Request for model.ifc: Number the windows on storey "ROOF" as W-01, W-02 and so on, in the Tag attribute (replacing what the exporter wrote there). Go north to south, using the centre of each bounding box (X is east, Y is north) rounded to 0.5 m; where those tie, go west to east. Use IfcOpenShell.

First a look at what the model holds.

```python
import ifcopenshell
import ifcopenshell.util.element
import ifcopenshell.util.placement

model = ifcopenshell.open("model.ifc")
print(model.schema)
storey = next(s for s in model.by_type("IfcBuildingStorey") if s.Name == "ROOF")
windows = [e for e in ifcopenshell.util.element.get_decomposition(storey) if e.is_a("IfcWindow")]
for e in sorted(windows, key=lambda e: e.id()):
    origin = ifcopenshell.util.placement.get_local_placement(e.ObjectPlacement)[:3, 3]
    print(e.id(), e.Tag, e.Name, origin.round(2) + 0.0, sep=" | ")
```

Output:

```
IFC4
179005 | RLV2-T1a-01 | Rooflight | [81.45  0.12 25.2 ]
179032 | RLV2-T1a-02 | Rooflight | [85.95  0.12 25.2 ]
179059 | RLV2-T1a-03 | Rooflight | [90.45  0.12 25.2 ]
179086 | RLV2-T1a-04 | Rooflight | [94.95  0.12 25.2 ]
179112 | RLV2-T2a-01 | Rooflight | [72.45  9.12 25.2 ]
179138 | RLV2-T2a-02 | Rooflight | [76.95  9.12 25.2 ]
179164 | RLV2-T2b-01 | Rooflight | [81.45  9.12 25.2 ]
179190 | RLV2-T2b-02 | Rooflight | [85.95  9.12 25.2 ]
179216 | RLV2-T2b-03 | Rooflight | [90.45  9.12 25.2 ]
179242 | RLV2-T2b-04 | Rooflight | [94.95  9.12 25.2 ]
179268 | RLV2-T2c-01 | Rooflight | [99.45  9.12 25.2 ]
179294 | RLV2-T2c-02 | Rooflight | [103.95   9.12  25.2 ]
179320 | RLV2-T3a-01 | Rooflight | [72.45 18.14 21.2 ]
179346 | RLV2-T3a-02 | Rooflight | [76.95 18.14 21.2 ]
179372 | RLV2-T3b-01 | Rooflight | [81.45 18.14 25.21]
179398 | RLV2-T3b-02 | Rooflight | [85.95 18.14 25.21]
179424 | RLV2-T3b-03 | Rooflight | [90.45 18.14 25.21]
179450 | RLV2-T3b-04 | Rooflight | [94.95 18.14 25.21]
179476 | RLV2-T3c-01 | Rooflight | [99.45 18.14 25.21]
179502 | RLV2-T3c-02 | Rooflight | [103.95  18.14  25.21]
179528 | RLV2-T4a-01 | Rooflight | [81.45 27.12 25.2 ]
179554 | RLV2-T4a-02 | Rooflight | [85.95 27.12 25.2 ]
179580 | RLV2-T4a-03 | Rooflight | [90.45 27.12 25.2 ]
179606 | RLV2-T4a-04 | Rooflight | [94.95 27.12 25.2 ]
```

```python
import ifcopenshell
import ifcopenshell.geom
import ifcopenshell.util.element
import ifcopenshell.util.shape

model = ifcopenshell.open("model.ifc")
settings = ifcopenshell.geom.settings()
settings.set("use-world-coords", True)


def centre(element):
    shape = ifcopenshell.geom.create_shape(settings, element)
    return ifcopenshell.util.shape.get_bbox_centroid(shape.geometry)


storey = next(s for s in model.by_type("IfcBuildingStorey") if s.Name == "ROOF")
windows = [e for e in ifcopenshell.util.element.get_decomposition(storey) if e.is_a("IfcWindow")]

# Insertion points can sit at a corner or the storey origin, so sort by the geometry (in metres).
centres = {e: centre(e) for e in windows}
windows.sort(key=lambda e: (-round(centres[e][1] / 0.5), centres[e][0]))

for i, e in enumerate(windows, start=1):
    number = f"W-{i:02d}"
    e.Tag = number
    print(e.id(), number)

model.write("model_updated.ifc")
```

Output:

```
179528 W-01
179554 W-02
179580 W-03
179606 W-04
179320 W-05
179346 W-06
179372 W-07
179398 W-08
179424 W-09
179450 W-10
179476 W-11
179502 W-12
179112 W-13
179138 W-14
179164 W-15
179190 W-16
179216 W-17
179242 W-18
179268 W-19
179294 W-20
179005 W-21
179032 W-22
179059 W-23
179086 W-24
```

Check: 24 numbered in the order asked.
